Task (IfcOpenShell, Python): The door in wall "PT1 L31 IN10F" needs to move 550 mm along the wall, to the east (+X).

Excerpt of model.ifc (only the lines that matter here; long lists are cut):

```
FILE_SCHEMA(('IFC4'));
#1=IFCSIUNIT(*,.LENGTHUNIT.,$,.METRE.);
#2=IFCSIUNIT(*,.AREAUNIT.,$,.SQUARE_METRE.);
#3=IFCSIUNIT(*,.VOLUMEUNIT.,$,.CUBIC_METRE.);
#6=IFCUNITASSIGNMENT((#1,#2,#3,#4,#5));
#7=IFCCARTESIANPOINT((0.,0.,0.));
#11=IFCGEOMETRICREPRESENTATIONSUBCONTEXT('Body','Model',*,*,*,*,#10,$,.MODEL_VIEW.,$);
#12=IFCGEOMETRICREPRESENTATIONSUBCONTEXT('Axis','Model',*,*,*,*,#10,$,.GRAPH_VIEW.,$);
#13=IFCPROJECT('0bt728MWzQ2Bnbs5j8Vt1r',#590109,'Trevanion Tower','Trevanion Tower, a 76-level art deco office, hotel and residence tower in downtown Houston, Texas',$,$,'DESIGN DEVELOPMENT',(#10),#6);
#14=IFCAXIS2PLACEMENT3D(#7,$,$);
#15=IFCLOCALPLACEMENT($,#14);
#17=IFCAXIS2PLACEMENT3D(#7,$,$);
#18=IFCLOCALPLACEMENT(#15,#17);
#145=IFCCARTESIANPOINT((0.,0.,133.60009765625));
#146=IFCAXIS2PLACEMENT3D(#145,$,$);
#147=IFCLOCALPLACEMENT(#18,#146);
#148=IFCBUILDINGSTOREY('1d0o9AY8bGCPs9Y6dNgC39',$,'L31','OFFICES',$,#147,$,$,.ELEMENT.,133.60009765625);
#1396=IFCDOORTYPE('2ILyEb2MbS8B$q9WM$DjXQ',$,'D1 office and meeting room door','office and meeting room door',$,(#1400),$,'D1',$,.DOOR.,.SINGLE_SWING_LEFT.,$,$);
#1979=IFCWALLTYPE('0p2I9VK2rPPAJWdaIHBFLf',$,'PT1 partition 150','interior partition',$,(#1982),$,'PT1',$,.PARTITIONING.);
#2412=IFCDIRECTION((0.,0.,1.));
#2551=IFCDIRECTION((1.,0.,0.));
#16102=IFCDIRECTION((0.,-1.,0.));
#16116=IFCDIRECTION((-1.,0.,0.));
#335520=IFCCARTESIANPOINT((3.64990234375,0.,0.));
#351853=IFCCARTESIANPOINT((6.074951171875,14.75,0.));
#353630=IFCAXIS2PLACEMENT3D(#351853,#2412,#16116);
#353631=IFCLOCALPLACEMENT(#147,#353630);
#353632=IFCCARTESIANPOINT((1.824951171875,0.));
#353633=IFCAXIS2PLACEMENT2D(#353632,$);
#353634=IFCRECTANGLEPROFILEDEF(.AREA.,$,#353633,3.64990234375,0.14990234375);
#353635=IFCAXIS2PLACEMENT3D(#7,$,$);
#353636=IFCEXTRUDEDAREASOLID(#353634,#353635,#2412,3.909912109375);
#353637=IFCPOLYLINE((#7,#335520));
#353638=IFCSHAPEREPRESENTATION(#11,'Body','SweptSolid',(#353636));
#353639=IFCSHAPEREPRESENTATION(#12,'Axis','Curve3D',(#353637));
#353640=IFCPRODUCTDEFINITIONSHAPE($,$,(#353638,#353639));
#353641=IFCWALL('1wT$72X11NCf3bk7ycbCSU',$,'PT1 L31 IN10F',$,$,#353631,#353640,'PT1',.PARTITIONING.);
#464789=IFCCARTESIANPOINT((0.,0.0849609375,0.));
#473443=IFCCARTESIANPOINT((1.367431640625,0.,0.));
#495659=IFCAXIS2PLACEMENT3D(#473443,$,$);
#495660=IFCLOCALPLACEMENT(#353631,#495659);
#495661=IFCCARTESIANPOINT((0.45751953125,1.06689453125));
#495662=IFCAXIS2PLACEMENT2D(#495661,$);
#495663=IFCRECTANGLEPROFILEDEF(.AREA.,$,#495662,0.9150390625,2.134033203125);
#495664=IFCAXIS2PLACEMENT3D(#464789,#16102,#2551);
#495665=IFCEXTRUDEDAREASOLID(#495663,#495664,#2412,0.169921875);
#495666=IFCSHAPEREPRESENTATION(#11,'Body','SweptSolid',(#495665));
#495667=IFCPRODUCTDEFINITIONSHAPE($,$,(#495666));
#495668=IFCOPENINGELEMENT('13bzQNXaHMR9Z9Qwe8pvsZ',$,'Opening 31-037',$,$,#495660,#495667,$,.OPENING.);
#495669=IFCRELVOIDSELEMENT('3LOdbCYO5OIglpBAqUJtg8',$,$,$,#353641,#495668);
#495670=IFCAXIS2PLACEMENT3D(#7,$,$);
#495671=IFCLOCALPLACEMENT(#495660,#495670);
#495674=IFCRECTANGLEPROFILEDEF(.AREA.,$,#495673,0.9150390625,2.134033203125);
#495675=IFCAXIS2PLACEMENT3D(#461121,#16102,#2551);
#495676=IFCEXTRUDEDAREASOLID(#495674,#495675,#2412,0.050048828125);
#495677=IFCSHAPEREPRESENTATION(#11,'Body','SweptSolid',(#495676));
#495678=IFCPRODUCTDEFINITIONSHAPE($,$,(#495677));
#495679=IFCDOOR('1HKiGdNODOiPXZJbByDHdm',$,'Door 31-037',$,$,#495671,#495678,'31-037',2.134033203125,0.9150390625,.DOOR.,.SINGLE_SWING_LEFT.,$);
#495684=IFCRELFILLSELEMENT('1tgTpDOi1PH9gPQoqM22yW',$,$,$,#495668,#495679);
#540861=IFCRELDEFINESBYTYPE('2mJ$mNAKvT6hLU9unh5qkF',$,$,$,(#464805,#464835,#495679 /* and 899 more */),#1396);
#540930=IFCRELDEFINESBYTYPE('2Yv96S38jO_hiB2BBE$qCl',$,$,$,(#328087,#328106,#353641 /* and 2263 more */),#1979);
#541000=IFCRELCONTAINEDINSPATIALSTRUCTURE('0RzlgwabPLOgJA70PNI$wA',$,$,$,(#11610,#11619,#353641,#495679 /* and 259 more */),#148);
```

```python
import ifcopenshell
import ifcopenshell.api.geometry
import ifcopenshell.util.placement
import ifcopenshell.util.unit

model = ifcopenshell.open("model.ifc")
unit_scale = ifcopenshell.util.unit.calculate_unit_scale(model)

door = model.by_guid("1HKiGdNODOiPXZJbByDHdm")
opening = door.FillsVoids[0].RelatingOpeningElement
wall = opening.VoidsElements[0].RelatingBuildingElement

wall_matrix = ifcopenshell.util.placement.get_local_placement(wall.ObjectPlacement)
shift = wall_matrix[:3, 0] * -0.55 / unit_scale
before = ifcopenshell.util.placement.get_local_placement(door.ObjectPlacement)[:3, 3].copy()

# The door is placed relative to its opening, so it follows when the opening moves.
matrix = ifcopenshell.util.placement.get_local_placement(opening.ObjectPlacement)
matrix[:3, 3] += shift
ifcopenshell.api.geometry.edit_object_placement(
    model, product=opening, matrix=matrix, is_si=False, should_transform_children=True
)

after = ifcopenshell.util.placement.get_local_placement(door.ObjectPlacement)[:3, 3]
print("door moved by", (after - before).round(3) + 0.0)

model.write("model_edited.ifc")
```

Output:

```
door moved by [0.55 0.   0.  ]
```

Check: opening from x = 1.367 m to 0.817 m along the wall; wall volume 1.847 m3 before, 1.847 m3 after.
